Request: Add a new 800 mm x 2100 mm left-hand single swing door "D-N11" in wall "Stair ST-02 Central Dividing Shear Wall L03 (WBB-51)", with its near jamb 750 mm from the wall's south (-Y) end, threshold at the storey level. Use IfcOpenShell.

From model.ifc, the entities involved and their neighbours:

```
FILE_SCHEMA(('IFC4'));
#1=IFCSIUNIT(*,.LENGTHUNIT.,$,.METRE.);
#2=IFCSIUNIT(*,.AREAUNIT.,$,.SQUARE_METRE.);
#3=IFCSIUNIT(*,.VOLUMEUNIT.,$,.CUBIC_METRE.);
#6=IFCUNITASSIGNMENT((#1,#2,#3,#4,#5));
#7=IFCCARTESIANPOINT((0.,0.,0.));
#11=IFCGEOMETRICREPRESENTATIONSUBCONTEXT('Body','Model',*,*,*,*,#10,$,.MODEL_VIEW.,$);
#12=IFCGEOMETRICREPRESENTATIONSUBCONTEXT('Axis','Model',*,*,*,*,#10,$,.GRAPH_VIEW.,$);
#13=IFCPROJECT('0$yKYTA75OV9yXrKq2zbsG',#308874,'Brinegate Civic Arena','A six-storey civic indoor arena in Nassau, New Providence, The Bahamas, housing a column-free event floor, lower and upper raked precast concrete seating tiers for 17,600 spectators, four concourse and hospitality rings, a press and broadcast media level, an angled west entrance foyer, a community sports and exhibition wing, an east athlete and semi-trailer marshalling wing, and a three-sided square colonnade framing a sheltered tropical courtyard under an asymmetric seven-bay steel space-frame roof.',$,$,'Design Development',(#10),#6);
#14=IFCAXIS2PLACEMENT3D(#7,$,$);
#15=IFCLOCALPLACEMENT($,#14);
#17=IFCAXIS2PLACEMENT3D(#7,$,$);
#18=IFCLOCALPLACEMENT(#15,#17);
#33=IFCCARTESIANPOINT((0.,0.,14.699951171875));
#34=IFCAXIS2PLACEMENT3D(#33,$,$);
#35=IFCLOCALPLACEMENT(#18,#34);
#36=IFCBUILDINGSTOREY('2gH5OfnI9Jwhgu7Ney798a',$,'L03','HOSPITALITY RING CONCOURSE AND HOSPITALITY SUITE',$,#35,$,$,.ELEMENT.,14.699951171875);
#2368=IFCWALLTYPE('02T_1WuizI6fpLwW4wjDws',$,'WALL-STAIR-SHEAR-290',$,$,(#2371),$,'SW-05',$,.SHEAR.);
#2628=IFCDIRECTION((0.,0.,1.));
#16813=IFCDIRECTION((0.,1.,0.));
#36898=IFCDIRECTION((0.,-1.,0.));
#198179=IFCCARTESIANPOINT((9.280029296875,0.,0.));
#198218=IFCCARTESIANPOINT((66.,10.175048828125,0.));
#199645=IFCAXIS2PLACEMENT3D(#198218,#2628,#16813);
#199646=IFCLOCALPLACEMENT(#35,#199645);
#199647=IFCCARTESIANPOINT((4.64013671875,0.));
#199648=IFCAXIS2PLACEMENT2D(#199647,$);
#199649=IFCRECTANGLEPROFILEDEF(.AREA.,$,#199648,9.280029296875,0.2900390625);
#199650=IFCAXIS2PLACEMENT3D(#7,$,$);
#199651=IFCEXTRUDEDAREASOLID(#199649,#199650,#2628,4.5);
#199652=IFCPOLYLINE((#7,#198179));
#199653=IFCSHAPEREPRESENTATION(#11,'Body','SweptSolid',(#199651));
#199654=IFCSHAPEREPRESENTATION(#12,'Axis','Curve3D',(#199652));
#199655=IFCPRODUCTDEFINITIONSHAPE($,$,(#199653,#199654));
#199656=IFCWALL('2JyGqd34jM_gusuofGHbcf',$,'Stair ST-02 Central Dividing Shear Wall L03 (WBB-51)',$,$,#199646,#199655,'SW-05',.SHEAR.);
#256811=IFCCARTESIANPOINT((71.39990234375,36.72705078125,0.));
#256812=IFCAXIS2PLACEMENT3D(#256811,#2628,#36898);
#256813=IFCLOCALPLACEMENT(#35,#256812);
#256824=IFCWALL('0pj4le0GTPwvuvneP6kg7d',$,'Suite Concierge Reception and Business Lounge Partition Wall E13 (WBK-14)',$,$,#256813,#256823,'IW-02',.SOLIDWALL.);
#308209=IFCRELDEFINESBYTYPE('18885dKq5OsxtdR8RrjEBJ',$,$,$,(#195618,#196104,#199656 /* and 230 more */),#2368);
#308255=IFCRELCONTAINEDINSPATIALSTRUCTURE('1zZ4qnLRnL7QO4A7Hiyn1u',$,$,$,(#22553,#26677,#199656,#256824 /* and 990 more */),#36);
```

```python
import numpy as np
import ifcopenshell
import ifcopenshell.api.feature
import ifcopenshell.api.geometry
import ifcopenshell.api.root
import ifcopenshell.api.spatial
import ifcopenshell.geom
import ifcopenshell.util.element
import ifcopenshell.util.placement
import ifcopenshell.util.representation
import ifcopenshell.util.shape
import ifcopenshell.util.unit

model = ifcopenshell.open("model.ifc")
unit_scale = ifcopenshell.util.unit.calculate_unit_scale(model)
settings = ifcopenshell.geom.settings()


def volume(element):
    """Net volume in cubic metres, openings subtracted."""
    shape = ifcopenshell.geom.create_shape(settings, element)
    return ifcopenshell.util.shape.get_volume(shape.geometry)


wall = model.by_id(199656)
storey = ifcopenshell.util.element.get_container(wall, ifc_class="IfcBuildingStorey")
context = ifcopenshell.util.representation.get_context(model, "Model", "Body", "MODEL_VIEW")
before = volume(wall)

width, height, from_end, sill = 0.8, 2.1, 0.75, 0.0  # metres

# The wall runs along its own X axis, and the end named is its -X end.
wall_shape = ifcopenshell.geom.create_shape(settings, wall)
x, y, z = ifcopenshell.util.shape.get_vertices(wall_shape.geometry).T
start = x.min() + from_end
face, thickness = float(y.min()), float(y.max() - y.min())
wall_matrix = ifcopenshell.util.placement.get_local_placement(wall.ObjectPlacement)
level = ifcopenshell.util.placement.get_local_placement(storey.ObjectPlacement)[2, 3]


def in_wall(x, y):
    """Placement at x, y metres in the wall's axes, at sill height."""
    matrix = wall_matrix.copy()
    matrix[:, 3] = wall_matrix @ np.array([x / unit_scale, y / unit_scale, 0.0, 1.0])
    matrix[2, 3] = level + sill / unit_scale
    return matrix


# Opening: a box that overshoots both wall faces by 50 mm.
opening = ifcopenshell.api.root.create_entity(model, ifc_class="IfcOpeningElement", predefined_type="OPENING")
box = ifcopenshell.api.geometry.add_wall_representation(
    model, context=context, length=width, height=height, thickness=thickness + 0.1
)
ifcopenshell.api.geometry.assign_representation(model, product=opening, representation=box)
ifcopenshell.api.geometry.edit_object_placement(model, product=opening, matrix=in_wall(start, face - 0.05), is_si=False)
ifcopenshell.api.feature.add_feature(model, feature=opening, element=wall)

door = ifcopenshell.api.root.create_entity(model, ifc_class="IfcDoor", name="D-N11", predefined_type="DOOR")
door.OverallWidth, door.OverallHeight = width / unit_scale, height / unit_scale
door.OperationType = "SINGLE_SWING_LEFT"
body = ifcopenshell.api.geometry.add_door_representation(
    model,
    context=context,
    overall_width=door.OverallWidth,
    overall_height=door.OverallHeight,
    operation_type="SINGLE_SWING_LEFT",
    lining_properties={"LiningDepth": thickness / unit_scale, "ThresholdDepth": thickness / unit_scale},
)
ifcopenshell.api.geometry.assign_representation(model, product=door, representation=body)
ifcopenshell.api.spatial.assign_container(model, products=[door], relating_structure=storey)
ifcopenshell.api.feature.add_filling(model, opening=opening, element=door)

# The lining spans the wall, so the door starts at the wall face.
ifcopenshell.api.geometry.edit_object_placement(model, product=door, matrix=in_wall(start, face), is_si=False)

after = volume(wall)

print(f"wall volume {before:.3f} -> {after:.3f} m3")

model.write("model_v2.ifc")
```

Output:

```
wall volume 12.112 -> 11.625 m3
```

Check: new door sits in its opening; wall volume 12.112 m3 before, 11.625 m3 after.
